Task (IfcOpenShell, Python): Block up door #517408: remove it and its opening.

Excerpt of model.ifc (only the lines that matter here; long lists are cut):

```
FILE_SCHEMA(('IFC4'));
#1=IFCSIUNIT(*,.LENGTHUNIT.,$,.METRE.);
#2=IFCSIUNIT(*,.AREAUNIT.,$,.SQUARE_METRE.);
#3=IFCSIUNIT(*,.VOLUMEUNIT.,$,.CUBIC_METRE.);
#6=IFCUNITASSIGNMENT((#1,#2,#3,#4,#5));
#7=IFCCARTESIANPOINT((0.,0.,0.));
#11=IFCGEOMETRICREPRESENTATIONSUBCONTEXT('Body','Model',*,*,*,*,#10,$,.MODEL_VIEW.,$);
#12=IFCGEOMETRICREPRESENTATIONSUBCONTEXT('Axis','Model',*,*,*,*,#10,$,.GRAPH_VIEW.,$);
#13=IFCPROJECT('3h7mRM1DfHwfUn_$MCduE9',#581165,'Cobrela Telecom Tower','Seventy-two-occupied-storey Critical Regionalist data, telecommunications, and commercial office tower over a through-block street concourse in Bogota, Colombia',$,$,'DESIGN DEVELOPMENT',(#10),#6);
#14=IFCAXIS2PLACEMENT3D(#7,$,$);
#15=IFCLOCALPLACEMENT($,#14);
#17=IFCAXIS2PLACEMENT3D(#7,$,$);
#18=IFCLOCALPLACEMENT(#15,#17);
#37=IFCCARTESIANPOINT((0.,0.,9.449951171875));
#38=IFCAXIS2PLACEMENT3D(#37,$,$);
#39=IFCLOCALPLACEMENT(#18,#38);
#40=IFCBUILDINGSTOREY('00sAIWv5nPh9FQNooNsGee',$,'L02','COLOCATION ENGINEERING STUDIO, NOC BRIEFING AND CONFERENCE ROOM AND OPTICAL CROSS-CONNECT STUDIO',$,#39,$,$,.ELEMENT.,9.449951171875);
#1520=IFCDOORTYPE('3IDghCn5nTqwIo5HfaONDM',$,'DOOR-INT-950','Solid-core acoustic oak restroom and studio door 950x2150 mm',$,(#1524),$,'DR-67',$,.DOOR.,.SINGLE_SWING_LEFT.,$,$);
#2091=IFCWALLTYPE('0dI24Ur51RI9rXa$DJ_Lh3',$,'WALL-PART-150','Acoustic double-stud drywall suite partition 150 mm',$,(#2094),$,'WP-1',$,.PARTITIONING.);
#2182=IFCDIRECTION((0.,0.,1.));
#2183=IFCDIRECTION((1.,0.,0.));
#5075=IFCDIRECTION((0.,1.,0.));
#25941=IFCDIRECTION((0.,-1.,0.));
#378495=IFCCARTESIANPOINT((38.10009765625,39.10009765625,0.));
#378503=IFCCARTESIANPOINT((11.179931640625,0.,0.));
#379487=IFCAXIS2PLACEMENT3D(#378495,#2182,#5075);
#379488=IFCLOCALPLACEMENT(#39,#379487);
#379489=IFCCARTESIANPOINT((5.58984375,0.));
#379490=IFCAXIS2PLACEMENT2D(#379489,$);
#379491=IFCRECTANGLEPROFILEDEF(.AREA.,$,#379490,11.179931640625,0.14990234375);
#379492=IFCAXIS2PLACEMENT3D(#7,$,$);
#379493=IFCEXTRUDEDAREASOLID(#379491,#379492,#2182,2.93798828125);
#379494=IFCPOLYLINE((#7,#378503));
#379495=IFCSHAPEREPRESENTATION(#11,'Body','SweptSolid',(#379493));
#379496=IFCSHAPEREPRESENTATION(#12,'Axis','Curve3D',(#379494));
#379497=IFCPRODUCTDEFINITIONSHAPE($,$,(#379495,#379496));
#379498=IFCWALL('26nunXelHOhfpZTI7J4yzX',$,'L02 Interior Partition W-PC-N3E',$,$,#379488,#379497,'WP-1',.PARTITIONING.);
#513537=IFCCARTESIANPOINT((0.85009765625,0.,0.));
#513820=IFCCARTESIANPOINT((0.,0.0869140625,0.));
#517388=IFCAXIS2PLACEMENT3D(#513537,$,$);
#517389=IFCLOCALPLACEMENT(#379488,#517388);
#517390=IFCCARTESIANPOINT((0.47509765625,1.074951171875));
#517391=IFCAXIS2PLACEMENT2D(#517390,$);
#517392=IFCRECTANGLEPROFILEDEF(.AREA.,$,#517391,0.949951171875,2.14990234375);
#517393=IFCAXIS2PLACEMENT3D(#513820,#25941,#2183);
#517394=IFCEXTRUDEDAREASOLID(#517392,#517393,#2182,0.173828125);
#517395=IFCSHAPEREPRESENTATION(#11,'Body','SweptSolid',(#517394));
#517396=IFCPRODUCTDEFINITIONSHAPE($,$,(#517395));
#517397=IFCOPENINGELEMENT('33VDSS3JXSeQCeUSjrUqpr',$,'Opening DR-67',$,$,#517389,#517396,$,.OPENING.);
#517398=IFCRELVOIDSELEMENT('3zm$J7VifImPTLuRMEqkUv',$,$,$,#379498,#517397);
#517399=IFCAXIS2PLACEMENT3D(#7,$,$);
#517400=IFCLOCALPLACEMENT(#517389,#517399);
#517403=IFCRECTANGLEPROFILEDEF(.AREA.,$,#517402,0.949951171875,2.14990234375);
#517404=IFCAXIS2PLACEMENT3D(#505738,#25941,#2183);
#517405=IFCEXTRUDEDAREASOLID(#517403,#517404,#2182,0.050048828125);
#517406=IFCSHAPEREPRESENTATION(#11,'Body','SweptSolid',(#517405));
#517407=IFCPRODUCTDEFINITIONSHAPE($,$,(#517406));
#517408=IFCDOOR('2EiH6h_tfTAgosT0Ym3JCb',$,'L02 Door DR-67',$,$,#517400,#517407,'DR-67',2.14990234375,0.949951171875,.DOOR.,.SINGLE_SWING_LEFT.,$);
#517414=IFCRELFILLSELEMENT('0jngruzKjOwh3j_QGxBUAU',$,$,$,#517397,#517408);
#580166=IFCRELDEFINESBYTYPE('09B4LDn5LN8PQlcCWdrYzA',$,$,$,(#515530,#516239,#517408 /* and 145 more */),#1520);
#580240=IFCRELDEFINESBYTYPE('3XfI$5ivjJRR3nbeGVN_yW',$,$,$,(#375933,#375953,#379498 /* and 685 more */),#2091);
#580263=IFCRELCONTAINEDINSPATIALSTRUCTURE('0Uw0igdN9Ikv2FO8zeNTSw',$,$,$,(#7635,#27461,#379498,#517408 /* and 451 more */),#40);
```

```python
import ifcopenshell
import ifcopenshell.api.feature
import ifcopenshell.api.root
import ifcopenshell.geom
import ifcopenshell.util.shape

model = ifcopenshell.open("model.ifc")
settings = ifcopenshell.geom.settings()


def volume(element):
    """Net volume in cubic metres, openings subtracted."""
    shape = ifcopenshell.geom.create_shape(settings, element)
    return ifcopenshell.util.shape.get_volume(shape.geometry)


door = model.by_id(517408)
opening = door.FillsVoids[0].RelatingOpeningElement
wall = opening.VoidsElements[0].RelatingBuildingElement
before = volume(wall)

ifcopenshell.api.root.remove_product(model, product=door)
ifcopenshell.api.feature.remove_feature(model, feature=opening)

after = volume(wall)

print(f"wall volume {before:.3f} -> {after:.3f} m3")

model.write("model-out.ifc")
```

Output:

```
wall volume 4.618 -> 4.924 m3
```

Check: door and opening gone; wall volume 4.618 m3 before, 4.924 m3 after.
